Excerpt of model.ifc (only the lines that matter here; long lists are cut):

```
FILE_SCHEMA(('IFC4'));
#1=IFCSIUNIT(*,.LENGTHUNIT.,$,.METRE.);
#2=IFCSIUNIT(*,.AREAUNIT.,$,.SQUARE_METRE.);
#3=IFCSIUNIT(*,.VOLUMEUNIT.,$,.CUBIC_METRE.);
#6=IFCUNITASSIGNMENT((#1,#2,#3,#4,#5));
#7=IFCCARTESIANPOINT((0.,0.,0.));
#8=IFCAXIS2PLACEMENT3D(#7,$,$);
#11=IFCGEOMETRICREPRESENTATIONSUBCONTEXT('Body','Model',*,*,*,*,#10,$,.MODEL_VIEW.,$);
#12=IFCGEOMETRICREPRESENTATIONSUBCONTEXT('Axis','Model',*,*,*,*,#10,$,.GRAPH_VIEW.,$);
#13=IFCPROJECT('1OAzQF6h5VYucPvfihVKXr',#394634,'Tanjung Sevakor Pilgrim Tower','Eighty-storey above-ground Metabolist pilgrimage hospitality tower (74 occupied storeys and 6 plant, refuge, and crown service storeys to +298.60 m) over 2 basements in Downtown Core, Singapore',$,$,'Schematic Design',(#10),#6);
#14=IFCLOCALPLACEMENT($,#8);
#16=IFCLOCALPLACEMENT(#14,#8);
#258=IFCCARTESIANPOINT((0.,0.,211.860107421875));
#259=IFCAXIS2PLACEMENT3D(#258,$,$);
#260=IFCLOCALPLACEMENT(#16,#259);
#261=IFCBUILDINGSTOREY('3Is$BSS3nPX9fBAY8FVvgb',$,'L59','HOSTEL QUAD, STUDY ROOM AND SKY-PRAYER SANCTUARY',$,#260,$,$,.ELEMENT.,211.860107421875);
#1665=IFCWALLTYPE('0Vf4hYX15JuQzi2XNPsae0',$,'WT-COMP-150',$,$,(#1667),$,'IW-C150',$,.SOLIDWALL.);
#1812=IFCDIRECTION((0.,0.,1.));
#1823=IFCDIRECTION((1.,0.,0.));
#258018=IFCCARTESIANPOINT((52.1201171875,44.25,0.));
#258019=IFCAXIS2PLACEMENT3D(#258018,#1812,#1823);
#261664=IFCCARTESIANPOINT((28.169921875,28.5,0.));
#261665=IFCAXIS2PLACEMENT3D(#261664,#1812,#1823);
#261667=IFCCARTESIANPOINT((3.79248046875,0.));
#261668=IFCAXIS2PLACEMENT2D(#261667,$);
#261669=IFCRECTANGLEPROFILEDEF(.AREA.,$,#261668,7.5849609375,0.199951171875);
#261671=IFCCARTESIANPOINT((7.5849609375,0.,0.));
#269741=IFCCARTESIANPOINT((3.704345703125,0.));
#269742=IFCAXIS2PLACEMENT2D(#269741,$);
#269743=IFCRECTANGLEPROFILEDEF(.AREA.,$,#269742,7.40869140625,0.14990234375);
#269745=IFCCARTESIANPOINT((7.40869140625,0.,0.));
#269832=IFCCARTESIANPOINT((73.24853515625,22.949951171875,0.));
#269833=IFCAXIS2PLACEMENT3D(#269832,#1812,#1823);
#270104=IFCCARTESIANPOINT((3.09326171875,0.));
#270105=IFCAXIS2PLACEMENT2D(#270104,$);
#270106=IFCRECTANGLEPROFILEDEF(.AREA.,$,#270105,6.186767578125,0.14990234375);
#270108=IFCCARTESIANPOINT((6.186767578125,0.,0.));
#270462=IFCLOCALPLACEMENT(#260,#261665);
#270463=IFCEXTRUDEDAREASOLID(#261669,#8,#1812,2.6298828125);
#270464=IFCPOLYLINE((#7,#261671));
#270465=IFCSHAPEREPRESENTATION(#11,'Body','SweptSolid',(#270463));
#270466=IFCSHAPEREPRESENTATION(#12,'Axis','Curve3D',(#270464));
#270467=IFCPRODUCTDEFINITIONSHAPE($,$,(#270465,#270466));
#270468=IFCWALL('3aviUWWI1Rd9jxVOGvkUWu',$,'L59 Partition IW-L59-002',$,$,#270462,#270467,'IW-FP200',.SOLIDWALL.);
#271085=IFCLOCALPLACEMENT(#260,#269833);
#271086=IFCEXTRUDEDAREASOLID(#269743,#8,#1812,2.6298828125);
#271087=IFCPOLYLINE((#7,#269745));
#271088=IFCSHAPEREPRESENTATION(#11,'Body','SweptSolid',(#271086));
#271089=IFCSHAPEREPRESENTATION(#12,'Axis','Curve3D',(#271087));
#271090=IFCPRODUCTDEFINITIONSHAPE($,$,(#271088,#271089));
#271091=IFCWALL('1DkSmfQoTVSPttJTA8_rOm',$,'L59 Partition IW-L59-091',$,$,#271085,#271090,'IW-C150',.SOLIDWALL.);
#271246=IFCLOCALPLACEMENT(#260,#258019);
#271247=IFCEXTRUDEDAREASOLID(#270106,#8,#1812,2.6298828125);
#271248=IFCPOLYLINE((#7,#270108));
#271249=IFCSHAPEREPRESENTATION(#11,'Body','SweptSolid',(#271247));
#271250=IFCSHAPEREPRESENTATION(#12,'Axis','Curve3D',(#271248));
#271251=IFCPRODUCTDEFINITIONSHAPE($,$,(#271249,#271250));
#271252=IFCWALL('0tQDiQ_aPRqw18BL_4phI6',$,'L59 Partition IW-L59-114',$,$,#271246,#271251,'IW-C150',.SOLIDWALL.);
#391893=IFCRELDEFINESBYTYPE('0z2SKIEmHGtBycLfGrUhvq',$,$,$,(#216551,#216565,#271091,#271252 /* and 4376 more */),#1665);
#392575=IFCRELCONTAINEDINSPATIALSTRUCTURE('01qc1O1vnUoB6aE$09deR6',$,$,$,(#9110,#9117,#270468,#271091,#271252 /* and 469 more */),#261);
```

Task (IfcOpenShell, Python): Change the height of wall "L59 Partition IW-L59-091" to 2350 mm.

```python
import ifcopenshell
import ifcopenshell.geom
import ifcopenshell.util.representation
import ifcopenshell.util.shape
import ifcopenshell.util.unit

model = ifcopenshell.open("model.ifc")
unit_scale = ifcopenshell.util.unit.calculate_unit_scale(model)
settings = ifcopenshell.geom.settings()


def volume(element):
    """Net volume in cubic metres, openings subtracted."""
    shape = ifcopenshell.geom.create_shape(settings, element)
    return ifcopenshell.util.shape.get_volume(shape.geometry)


wall = model.by_guid("1DkSmfQoTVSPttJTA8_rOm")
before = volume(wall)

body = ifcopenshell.util.representation.get_representation(wall, "Model", "Body")
solid = body.Items[0]
old_height = solid.Depth
solid.Depth = 2.35 / unit_scale
after = volume(wall)

print(f"height {old_height:g} -> {solid.Depth:g}, volume {before:.3f} -> {after:.3f} m3")

model.write("model_rev.ifc")
```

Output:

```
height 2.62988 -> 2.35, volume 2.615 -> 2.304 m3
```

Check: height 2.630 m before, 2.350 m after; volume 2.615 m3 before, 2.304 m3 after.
